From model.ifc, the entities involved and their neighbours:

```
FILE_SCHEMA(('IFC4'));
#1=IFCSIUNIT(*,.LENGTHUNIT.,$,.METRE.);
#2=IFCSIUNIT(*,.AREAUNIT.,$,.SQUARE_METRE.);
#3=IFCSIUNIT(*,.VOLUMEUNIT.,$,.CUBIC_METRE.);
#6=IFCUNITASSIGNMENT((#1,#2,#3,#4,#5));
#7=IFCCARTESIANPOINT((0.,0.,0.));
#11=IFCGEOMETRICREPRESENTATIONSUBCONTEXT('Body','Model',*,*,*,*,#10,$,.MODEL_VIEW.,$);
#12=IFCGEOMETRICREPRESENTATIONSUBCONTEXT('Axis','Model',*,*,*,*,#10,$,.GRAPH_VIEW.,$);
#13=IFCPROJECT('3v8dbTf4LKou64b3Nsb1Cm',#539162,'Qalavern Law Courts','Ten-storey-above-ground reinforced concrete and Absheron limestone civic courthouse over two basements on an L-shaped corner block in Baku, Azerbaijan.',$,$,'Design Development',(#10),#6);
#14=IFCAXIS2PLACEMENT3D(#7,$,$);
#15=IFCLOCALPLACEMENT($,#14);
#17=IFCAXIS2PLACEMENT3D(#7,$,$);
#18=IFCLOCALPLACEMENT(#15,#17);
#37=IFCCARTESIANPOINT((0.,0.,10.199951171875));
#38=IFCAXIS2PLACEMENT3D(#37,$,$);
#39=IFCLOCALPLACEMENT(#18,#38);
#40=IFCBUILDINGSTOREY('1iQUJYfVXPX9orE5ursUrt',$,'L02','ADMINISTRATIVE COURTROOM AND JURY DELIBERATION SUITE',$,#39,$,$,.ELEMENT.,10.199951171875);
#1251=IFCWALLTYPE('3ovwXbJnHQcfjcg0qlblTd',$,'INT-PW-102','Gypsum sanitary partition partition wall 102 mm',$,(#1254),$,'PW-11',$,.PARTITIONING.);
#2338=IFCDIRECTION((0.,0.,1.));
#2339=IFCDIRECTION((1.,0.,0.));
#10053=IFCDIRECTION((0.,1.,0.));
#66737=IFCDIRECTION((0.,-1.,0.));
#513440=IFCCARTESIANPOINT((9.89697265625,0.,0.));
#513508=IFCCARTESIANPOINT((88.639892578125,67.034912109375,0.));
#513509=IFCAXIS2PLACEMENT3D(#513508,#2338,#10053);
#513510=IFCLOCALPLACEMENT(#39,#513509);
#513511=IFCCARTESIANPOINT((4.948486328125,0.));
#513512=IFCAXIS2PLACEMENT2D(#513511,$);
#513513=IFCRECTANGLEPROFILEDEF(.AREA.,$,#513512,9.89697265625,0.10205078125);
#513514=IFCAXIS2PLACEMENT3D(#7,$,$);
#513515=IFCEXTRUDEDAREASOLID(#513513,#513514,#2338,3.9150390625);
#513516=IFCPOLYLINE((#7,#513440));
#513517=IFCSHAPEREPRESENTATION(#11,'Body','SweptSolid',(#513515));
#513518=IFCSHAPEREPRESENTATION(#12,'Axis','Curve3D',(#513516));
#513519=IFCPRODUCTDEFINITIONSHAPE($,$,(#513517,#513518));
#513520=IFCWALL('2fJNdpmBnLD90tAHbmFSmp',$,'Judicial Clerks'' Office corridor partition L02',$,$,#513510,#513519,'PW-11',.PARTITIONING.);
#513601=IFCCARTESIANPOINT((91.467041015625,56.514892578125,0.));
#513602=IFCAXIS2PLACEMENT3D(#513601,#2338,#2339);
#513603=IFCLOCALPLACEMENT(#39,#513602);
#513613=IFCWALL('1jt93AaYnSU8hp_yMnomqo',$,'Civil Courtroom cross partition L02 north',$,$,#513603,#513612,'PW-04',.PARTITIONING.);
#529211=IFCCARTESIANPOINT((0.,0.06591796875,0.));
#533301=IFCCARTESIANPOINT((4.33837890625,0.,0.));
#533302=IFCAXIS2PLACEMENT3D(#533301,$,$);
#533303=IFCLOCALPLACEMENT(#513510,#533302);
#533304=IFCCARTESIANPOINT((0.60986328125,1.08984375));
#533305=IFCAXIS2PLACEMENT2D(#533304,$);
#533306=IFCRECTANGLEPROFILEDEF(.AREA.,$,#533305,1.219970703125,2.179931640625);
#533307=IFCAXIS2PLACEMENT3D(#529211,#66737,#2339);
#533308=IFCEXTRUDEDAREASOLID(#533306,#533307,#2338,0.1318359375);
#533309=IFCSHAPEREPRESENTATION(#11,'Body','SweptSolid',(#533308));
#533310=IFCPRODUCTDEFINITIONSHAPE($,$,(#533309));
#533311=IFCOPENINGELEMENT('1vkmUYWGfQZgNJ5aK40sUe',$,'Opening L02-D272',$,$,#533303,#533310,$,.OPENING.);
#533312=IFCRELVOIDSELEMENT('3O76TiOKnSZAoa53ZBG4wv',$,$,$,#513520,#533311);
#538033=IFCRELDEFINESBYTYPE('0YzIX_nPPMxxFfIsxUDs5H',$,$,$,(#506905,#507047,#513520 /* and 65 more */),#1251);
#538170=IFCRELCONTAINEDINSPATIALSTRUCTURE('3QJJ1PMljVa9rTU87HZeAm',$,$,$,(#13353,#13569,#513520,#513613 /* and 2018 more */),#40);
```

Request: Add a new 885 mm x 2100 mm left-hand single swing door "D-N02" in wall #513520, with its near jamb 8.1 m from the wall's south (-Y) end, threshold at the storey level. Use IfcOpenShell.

```python
import numpy as np
import ifcopenshell
import ifcopenshell.api.feature
import ifcopenshell.api.geometry
import ifcopenshell.api.root
import ifcopenshell.api.spatial
import ifcopenshell.geom
import ifcopenshell.util.element
import ifcopenshell.util.placement
import ifcopenshell.util.representation
import ifcopenshell.util.shape
import ifcopenshell.util.unit

model = ifcopenshell.open("model.ifc")
unit_scale = ifcopenshell.util.unit.calculate_unit_scale(model)
settings = ifcopenshell.geom.settings()


def volume(element):
    """Net volume in cubic metres, openings subtracted."""
    shape = ifcopenshell.geom.create_shape(settings, element)
    return ifcopenshell.util.shape.get_volume(shape.geometry)


wall = model.by_guid("2fJNdpmBnLD90tAHbmFSmp")
storey = ifcopenshell.util.element.get_container(wall, ifc_class="IfcBuildingStorey")
context = ifcopenshell.util.representation.get_context(model, "Model", "Body", "MODEL_VIEW")
before = volume(wall)

width, height, from_end, sill = 0.885, 2.1, 8.1, 0.0  # metres

# The wall runs along its own X axis, and the end named is its -X end.
wall_shape = ifcopenshell.geom.create_shape(settings, wall)
x, y, z = ifcopenshell.util.shape.get_vertices(wall_shape.geometry).T
start = x.min() + from_end
face, thickness = float(y.min()), float(y.max() - y.min())
wall_matrix = ifcopenshell.util.placement.get_local_placement(wall.ObjectPlacement)
level = ifcopenshell.util.placement.get_local_placement(storey.ObjectPlacement)[2, 3]


def in_wall(x, y):
    """Placement at x, y metres in the wall's axes, at sill height."""
    matrix = wall_matrix.copy()
    matrix[:, 3] = wall_matrix @ np.array([x / unit_scale, y / unit_scale, 0.0, 1.0])
    matrix[2, 3] = level + sill / unit_scale
    return matrix


# Opening: a box that overshoots both wall faces by 50 mm.
opening = ifcopenshell.api.root.create_entity(model, ifc_class="IfcOpeningElement", predefined_type="OPENING")
box = ifcopenshell.api.geometry.add_wall_representation(
    model, context=context, length=width, height=height, thickness=thickness + 0.1
)
ifcopenshell.api.geometry.assign_representation(model, product=opening, representation=box)
ifcopenshell.api.geometry.edit_object_placement(model, product=opening, matrix=in_wall(start, face - 0.05), is_si=False)
ifcopenshell.api.feature.add_feature(model, feature=opening, element=wall)

door = ifcopenshell.api.root.create_entity(model, ifc_class="IfcDoor", name="D-N02", predefined_type="DOOR")
door.OverallWidth, door.OverallHeight = width / unit_scale, height / unit_scale
door.OperationType = "SINGLE_SWING_LEFT"
body = ifcopenshell.api.geometry.add_door_representation(
    model,
    context=context,
    overall_width=door.OverallWidth,
    overall_height=door.OverallHeight,
    operation_type="SINGLE_SWING_LEFT",
    lining_properties={"LiningDepth": thickness / unit_scale, "ThresholdDepth": thickness / unit_scale},
)
ifcopenshell.api.geometry.assign_representation(model, product=door, representation=body)
ifcopenshell.api.spatial.assign_container(model, products=[door], relating_structure=storey)
ifcopenshell.api.feature.add_filling(model, opening=opening, element=door)

# The lining spans the wall, so the door starts at the wall face.
ifcopenshell.api.geometry.edit_object_placement(model, product=door, matrix=in_wall(start, face), is_si=False)

after = volume(wall)

print(f"wall volume {before:.3f} -> {after:.3f} m3")

model.write("model-out.ifc")
```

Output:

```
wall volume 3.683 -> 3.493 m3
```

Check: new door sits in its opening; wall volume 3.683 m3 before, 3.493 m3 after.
